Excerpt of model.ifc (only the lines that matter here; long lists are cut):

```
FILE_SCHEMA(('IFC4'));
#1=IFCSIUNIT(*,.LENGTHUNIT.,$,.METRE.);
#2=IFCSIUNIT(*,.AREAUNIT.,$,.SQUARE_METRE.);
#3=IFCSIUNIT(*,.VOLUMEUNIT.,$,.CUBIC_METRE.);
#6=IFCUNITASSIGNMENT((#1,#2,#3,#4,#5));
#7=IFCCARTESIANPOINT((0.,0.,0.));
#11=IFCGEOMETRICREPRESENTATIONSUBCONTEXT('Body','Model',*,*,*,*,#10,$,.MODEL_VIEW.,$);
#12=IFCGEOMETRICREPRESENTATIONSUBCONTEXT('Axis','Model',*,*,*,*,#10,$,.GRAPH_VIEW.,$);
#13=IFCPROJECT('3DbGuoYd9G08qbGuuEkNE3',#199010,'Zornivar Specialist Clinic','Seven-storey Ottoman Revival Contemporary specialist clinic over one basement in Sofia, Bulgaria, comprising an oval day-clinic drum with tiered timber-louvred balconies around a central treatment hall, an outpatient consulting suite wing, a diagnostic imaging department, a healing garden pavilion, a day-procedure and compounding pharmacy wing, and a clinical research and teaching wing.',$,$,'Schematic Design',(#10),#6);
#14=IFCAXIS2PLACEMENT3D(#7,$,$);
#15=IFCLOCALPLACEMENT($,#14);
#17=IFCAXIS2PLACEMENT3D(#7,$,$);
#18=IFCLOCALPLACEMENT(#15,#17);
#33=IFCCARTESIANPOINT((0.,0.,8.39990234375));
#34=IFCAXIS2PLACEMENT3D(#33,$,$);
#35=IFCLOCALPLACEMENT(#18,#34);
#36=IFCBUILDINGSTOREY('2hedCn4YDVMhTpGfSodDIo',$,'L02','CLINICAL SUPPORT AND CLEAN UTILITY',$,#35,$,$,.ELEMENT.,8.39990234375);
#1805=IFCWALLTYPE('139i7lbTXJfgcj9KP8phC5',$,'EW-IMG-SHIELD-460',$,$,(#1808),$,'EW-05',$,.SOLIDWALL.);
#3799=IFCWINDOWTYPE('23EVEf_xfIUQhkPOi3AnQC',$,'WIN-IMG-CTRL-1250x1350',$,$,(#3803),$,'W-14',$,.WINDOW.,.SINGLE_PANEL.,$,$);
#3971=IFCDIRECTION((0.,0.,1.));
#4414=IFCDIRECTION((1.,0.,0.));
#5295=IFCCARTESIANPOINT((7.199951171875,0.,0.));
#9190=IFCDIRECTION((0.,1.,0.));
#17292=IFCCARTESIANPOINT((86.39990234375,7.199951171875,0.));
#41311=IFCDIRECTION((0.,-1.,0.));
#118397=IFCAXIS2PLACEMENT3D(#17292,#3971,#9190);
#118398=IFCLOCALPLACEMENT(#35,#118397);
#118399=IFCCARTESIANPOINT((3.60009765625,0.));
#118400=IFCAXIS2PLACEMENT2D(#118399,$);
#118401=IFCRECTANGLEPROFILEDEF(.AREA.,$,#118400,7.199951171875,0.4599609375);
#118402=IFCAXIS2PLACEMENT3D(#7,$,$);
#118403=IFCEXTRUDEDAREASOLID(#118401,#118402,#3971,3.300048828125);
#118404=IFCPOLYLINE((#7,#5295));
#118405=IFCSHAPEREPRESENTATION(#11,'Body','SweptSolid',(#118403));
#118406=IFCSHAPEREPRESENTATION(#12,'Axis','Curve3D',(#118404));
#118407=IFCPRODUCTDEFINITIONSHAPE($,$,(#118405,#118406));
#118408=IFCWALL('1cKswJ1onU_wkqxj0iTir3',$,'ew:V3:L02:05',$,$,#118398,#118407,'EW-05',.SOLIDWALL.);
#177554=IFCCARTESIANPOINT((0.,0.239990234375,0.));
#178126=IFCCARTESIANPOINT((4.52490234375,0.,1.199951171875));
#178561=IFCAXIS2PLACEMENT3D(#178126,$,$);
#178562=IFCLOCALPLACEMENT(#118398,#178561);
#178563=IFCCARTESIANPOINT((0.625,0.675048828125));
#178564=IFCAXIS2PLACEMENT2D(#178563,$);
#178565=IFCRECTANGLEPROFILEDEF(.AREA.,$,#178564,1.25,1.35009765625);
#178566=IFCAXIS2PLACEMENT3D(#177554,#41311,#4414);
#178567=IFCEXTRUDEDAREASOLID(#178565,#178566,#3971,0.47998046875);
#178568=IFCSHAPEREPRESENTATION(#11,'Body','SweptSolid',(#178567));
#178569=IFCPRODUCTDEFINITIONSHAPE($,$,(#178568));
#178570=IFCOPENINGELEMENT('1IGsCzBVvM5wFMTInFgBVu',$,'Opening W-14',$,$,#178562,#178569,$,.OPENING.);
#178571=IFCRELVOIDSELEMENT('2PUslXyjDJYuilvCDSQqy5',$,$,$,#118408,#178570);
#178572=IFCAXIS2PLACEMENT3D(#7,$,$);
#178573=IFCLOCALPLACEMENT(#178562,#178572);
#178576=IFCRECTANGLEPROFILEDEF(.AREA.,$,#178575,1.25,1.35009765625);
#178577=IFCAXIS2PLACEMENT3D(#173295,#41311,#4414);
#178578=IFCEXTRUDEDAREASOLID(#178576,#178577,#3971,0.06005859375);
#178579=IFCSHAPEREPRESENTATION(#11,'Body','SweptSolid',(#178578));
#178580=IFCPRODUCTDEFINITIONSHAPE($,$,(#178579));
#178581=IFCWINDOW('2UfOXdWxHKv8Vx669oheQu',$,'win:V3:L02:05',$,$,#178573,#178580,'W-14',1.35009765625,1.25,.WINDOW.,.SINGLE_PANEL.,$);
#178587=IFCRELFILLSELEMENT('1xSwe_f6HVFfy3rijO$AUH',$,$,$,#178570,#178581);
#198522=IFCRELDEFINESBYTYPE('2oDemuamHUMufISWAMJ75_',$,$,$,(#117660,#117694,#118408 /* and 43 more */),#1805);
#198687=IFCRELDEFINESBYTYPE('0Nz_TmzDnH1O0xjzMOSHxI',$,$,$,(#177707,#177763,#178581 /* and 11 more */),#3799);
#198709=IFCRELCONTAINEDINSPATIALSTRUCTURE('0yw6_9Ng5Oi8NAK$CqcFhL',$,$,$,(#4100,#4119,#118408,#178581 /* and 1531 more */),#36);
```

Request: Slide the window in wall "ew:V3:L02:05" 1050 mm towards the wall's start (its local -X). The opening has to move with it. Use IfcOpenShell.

```python
import ifcopenshell
import ifcopenshell.api.geometry
import ifcopenshell.util.placement
import ifcopenshell.util.unit

model = ifcopenshell.open("model.ifc")
unit_scale = ifcopenshell.util.unit.calculate_unit_scale(model)

window = model.by_guid("2UfOXdWxHKv8Vx669oheQu")
opening = window.FillsVoids[0].RelatingOpeningElement
wall = opening.VoidsElements[0].RelatingBuildingElement

wall_matrix = ifcopenshell.util.placement.get_local_placement(wall.ObjectPlacement)
shift = wall_matrix[:3, 0] * -1.05 / unit_scale
before = ifcopenshell.util.placement.get_local_placement(window.ObjectPlacement)[:3, 3].copy()

# The window is placed relative to its opening, so it follows when the opening moves.
matrix = ifcopenshell.util.placement.get_local_placement(opening.ObjectPlacement)
matrix[:3, 3] += shift
ifcopenshell.api.geometry.edit_object_placement(
    model, product=opening, matrix=matrix, is_si=False, should_transform_children=True
)

after = ifcopenshell.util.placement.get_local_placement(window.ObjectPlacement)[:3, 3]
print("window moved by", (after - before).round(3) + 0.0)

model.write("model_updated.ifc")
```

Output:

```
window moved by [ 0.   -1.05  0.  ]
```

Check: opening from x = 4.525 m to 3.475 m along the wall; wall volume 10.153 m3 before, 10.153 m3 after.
